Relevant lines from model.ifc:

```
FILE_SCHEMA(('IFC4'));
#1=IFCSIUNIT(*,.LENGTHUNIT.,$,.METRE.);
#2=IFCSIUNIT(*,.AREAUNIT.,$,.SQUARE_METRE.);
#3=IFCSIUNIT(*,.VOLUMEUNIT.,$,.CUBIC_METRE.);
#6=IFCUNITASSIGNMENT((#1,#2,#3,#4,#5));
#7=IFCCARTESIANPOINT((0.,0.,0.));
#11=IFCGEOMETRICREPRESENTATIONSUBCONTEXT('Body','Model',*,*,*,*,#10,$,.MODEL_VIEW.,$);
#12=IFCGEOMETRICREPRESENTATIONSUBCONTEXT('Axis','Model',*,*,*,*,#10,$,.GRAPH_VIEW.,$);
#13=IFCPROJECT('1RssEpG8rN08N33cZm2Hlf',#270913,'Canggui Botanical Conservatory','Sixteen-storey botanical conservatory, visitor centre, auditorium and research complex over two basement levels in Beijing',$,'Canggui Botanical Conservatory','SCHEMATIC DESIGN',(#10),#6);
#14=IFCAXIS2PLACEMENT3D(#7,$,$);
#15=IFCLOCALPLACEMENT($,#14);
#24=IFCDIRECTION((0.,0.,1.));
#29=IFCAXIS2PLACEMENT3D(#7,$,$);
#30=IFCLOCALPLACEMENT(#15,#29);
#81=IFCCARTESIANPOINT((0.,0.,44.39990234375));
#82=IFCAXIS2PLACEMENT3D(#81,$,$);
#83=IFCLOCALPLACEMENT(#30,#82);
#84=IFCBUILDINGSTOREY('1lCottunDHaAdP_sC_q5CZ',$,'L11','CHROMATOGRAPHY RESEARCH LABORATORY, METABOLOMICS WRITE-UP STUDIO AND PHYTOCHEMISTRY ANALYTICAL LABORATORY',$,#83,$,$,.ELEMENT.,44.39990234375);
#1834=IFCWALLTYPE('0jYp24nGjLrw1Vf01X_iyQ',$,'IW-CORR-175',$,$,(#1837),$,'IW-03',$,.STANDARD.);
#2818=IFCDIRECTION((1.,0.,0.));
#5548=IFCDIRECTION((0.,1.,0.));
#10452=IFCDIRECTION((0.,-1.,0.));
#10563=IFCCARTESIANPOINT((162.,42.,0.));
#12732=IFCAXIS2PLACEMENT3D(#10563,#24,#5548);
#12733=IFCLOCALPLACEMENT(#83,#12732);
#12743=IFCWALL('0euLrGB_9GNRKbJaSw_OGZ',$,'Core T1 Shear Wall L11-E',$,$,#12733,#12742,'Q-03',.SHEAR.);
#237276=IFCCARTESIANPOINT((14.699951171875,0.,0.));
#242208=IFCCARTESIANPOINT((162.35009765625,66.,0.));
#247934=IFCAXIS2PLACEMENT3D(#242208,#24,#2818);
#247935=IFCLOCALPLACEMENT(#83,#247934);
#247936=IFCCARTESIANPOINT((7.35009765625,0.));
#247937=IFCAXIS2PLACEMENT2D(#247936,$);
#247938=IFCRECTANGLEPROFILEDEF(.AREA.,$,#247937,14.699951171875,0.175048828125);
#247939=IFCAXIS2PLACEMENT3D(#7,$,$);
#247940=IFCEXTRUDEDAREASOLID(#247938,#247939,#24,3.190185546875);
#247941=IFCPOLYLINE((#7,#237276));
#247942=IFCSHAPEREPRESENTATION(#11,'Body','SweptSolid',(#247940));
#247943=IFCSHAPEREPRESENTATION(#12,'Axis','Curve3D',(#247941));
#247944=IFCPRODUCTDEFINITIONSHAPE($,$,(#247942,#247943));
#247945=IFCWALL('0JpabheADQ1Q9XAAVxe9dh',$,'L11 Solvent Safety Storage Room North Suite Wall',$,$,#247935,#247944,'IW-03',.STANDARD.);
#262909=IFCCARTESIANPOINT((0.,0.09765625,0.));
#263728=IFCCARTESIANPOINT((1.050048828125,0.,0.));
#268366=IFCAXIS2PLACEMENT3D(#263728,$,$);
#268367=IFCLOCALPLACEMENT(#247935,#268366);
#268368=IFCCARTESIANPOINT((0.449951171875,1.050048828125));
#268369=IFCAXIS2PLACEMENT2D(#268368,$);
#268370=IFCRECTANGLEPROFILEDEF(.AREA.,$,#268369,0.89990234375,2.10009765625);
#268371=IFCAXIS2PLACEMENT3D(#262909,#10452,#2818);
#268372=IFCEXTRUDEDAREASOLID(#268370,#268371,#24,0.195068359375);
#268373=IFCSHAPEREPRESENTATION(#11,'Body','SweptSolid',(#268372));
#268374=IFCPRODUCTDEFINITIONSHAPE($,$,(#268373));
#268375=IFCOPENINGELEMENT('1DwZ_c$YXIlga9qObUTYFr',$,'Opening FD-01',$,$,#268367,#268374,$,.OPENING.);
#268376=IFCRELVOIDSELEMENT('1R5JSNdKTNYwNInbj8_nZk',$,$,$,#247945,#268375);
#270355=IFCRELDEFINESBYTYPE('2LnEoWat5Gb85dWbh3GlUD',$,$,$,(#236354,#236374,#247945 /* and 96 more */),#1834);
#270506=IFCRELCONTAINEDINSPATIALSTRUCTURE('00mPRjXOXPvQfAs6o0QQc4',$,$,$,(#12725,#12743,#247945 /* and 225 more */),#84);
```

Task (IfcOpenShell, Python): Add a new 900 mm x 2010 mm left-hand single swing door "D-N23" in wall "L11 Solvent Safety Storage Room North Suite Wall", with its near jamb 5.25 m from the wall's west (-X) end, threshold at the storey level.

```python
import numpy as np
import ifcopenshell
import ifcopenshell.api.feature
import ifcopenshell.api.geometry
import ifcopenshell.api.root
import ifcopenshell.api.spatial
import ifcopenshell.geom
import ifcopenshell.util.element
import ifcopenshell.util.placement
import ifcopenshell.util.representation
import ifcopenshell.util.shape
import ifcopenshell.util.unit

model = ifcopenshell.open("model.ifc")
unit_scale = ifcopenshell.util.unit.calculate_unit_scale(model)
settings = ifcopenshell.geom.settings()


def volume(element):
    """Net volume in cubic metres, openings subtracted."""
    shape = ifcopenshell.geom.create_shape(settings, element)
    return ifcopenshell.util.shape.get_volume(shape.geometry)


wall = model.by_id(247945)
storey = ifcopenshell.util.element.get_container(wall, ifc_class="IfcBuildingStorey")
context = ifcopenshell.util.representation.get_context(model, "Model", "Body", "MODEL_VIEW")
before = volume(wall)

width, height, from_end, sill = 0.9, 2.01, 5.25, 0.0  # metres

# The wall runs along its own X axis, and the end named is its -X end.
wall_shape = ifcopenshell.geom.create_shape(settings, wall)
x, y, z = ifcopenshell.util.shape.get_vertices(wall_shape.geometry).T
start = x.min() + from_end
face, thickness = float(y.min()), float(y.max() - y.min())
wall_matrix = ifcopenshell.util.placement.get_local_placement(wall.ObjectPlacement)
level = ifcopenshell.util.placement.get_local_placement(storey.ObjectPlacement)[2, 3]


def in_wall(x, y):
    """Placement at x, y metres in the wall's axes, at sill height."""
    matrix = wall_matrix.copy()
    matrix[:, 3] = wall_matrix @ np.array([x / unit_scale, y / unit_scale, 0.0, 1.0])
    matrix[2, 3] = level + sill / unit_scale
    return matrix


# Opening: a box that overshoots both wall faces by 50 mm.
opening = ifcopenshell.api.root.create_entity(model, ifc_class="IfcOpeningElement", predefined_type="OPENING")
box = ifcopenshell.api.geometry.add_wall_representation(
    model, context=context, length=width, height=height, thickness=thickness + 0.1
)
ifcopenshell.api.geometry.assign_representation(model, product=opening, representation=box)
ifcopenshell.api.geometry.edit_object_placement(model, product=opening, matrix=in_wall(start, face - 0.05), is_si=False)
ifcopenshell.api.feature.add_feature(model, feature=opening, element=wall)

door = ifcopenshell.api.root.create_entity(model, ifc_class="IfcDoor", name="D-N23", predefined_type="DOOR")
door.OverallWidth, door.OverallHeight = width / unit_scale, height / unit_scale
door.OperationType = "SINGLE_SWING_LEFT"
body = ifcopenshell.api.geometry.add_door_representation(
    model,
    context=context,
    overall_width=door.OverallWidth,
    overall_height=door.OverallHeight,
    operation_type="SINGLE_SWING_LEFT",
    lining_properties={"LiningDepth": thickness / unit_scale, "ThresholdDepth": thickness / unit_scale},
)
ifcopenshell.api.geometry.assign_representation(model, product=door, representation=body)
ifcopenshell.api.spatial.assign_container(model, products=[door], relating_structure=storey)
ifcopenshell.api.feature.add_filling(model, opening=opening, element=door)

# The lining spans the wall, so the door starts at the wall face.
ifcopenshell.api.geometry.edit_object_placement(model, product=door, matrix=in_wall(start, face), is_si=False)

after = volume(wall)

print(f"wall volume {before:.3f} -> {after:.3f} m3")

model.write("model_updated.ifc")
```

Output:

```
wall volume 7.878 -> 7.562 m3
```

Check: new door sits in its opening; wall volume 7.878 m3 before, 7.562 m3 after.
